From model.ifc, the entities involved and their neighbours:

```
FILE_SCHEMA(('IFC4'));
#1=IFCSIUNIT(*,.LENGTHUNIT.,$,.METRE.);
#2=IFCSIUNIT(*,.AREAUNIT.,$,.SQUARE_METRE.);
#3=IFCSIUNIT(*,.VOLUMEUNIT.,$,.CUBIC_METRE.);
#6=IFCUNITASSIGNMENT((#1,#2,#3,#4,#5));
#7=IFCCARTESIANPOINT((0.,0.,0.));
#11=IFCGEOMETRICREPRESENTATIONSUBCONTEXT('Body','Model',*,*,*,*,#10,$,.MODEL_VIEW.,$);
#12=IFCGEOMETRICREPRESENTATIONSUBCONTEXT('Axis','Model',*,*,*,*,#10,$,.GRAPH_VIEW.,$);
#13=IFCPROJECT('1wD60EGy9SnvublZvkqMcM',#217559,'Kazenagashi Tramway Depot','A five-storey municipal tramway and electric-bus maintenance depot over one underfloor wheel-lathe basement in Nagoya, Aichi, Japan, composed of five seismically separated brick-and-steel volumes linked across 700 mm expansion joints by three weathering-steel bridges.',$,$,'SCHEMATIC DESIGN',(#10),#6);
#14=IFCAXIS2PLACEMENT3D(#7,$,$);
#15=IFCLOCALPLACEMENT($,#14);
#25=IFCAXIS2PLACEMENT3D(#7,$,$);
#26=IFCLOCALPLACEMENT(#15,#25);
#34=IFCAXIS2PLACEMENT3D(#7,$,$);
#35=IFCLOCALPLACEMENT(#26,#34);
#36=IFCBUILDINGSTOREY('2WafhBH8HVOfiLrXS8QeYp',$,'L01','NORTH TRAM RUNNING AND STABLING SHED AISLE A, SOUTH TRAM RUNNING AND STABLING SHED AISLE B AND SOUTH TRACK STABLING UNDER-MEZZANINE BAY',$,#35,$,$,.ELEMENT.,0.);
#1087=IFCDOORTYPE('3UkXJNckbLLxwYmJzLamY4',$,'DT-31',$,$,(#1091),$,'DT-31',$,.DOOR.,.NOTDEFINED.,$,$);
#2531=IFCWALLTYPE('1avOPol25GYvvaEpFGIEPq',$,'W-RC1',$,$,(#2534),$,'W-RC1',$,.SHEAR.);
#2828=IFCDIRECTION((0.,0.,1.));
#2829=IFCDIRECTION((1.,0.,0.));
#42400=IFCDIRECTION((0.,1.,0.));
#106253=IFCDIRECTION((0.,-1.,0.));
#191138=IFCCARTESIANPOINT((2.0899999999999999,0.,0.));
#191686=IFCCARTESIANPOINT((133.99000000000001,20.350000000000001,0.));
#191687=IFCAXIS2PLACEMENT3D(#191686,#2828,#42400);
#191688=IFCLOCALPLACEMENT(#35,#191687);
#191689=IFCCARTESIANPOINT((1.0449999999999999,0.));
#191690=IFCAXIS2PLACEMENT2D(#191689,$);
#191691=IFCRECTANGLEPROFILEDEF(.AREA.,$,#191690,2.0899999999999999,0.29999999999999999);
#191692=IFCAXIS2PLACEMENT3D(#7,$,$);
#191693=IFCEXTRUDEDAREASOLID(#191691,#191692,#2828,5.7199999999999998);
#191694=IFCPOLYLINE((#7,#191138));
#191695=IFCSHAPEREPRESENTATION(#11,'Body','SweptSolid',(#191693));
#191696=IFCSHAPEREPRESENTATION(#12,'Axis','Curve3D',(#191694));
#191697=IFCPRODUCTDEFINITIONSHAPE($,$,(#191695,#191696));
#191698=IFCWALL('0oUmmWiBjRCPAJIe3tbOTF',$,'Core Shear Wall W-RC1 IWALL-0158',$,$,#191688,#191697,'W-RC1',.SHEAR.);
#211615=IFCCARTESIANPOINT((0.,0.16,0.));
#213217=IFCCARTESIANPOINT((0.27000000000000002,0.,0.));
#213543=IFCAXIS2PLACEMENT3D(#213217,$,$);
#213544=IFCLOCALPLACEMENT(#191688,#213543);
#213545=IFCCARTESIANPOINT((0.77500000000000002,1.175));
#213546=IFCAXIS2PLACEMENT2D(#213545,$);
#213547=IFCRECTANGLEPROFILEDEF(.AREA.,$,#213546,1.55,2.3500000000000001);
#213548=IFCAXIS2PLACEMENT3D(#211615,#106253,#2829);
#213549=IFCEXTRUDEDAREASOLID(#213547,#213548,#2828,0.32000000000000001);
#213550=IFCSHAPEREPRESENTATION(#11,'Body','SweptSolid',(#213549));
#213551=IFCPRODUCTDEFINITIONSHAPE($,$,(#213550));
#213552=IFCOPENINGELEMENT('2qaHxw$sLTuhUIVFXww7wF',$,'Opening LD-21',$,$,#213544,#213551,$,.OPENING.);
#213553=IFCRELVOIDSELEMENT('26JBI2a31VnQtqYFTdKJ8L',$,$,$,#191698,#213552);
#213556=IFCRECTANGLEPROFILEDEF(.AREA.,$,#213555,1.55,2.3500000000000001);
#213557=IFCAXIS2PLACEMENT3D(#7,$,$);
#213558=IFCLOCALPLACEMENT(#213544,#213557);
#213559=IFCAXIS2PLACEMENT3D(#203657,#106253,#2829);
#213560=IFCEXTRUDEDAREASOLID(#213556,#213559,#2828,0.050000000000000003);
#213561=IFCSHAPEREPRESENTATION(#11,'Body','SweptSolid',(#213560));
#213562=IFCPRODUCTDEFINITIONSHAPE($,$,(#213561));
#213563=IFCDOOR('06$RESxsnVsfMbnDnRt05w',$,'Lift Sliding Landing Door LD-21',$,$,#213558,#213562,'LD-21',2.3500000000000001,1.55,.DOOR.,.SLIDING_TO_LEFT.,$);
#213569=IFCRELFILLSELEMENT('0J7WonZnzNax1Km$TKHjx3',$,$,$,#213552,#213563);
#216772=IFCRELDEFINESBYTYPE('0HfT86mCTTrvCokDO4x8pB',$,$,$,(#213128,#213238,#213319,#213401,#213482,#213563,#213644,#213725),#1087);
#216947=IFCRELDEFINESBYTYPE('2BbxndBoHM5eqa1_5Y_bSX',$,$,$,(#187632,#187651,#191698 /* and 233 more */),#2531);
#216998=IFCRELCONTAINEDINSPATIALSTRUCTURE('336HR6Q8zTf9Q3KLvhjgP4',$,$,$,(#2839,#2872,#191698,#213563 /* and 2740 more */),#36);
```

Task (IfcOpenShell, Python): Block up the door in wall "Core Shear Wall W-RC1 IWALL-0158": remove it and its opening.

```python
import ifcopenshell
import ifcopenshell.api.feature
import ifcopenshell.api.root
import ifcopenshell.geom
import ifcopenshell.util.shape

model = ifcopenshell.open("model.ifc")
settings = ifcopenshell.geom.settings()


def volume(element):
    """Net volume in cubic metres, openings subtracted."""
    shape = ifcopenshell.geom.create_shape(settings, element)
    return ifcopenshell.util.shape.get_volume(shape.geometry)


door = model.by_guid("06$RESxsnVsfMbnDnRt05w")
opening = door.FillsVoids[0].RelatingOpeningElement
wall = opening.VoidsElements[0].RelatingBuildingElement
before = volume(wall)

ifcopenshell.api.root.remove_product(model, product=door)
ifcopenshell.api.feature.remove_feature(model, feature=opening)

after = volume(wall)

print(f"wall volume {before:.3f} -> {after:.3f} m3")

model.write("model_rev.ifc")
```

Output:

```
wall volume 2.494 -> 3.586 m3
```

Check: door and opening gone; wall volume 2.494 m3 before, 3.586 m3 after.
